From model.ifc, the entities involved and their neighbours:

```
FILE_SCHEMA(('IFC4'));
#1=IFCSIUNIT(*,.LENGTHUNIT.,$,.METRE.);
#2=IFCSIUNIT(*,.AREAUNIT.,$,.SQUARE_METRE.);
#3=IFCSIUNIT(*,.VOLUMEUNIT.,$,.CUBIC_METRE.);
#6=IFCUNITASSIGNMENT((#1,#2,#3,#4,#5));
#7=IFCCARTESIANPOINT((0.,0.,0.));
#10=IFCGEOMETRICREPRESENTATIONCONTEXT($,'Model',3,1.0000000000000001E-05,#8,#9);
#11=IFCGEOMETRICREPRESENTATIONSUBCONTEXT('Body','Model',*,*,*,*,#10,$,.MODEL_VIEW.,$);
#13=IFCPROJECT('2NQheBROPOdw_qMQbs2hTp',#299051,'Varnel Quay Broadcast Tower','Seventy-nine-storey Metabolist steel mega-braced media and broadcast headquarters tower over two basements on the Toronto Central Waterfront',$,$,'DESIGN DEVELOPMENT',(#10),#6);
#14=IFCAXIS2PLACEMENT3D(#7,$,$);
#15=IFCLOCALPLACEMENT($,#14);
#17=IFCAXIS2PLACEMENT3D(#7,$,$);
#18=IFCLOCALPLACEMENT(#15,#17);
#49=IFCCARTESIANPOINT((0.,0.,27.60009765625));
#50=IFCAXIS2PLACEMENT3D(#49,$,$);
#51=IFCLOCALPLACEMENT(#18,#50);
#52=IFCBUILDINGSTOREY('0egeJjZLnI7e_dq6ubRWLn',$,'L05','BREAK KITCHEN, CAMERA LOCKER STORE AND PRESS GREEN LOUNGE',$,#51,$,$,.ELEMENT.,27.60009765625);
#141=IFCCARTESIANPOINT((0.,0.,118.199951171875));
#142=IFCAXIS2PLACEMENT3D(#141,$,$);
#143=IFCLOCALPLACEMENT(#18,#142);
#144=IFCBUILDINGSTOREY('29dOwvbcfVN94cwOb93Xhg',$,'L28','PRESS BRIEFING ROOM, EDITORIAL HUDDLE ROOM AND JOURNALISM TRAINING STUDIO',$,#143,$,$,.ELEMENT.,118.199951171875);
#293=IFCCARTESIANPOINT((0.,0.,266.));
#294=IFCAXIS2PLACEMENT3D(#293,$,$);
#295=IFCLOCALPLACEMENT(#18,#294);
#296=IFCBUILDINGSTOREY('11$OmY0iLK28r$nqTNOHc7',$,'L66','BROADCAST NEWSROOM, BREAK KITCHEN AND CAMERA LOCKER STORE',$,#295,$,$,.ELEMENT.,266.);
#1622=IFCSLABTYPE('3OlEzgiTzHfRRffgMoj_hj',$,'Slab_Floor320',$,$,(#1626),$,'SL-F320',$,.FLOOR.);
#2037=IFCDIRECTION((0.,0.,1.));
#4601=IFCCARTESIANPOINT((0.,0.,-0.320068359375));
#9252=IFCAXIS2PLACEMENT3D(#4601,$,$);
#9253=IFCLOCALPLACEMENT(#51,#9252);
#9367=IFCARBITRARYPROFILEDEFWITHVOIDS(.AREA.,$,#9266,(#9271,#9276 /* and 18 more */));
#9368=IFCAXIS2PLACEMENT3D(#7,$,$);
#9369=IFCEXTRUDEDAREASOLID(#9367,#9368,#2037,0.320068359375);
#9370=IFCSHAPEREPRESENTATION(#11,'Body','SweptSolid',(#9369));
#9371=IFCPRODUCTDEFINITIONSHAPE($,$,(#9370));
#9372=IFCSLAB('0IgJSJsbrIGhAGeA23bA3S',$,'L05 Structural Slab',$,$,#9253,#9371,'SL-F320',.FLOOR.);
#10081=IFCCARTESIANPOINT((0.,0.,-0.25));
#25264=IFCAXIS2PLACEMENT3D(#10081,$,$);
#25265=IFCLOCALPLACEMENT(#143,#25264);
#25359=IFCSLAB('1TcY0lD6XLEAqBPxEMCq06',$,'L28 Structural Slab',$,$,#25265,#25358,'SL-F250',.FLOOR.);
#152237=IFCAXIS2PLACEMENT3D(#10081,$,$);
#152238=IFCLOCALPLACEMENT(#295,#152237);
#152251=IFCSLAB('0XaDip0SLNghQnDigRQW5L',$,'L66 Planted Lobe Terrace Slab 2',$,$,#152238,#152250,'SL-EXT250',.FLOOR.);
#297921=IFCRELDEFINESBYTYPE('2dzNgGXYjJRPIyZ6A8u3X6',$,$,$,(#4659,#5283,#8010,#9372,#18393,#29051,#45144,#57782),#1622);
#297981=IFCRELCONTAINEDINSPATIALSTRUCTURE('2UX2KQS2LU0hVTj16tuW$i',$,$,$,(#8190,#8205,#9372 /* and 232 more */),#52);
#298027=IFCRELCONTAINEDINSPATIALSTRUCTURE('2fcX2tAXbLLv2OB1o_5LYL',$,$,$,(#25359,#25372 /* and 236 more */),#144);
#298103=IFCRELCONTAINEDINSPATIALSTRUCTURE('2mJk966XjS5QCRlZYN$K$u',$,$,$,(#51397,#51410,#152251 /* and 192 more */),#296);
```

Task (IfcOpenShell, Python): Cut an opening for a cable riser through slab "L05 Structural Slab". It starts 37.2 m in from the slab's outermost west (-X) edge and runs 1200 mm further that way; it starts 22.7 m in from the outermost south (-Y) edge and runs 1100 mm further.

```python
import numpy as np
import ifcopenshell
import ifcopenshell.api.feature
import ifcopenshell.api.geometry
import ifcopenshell.api.root
import ifcopenshell.geom
import ifcopenshell.util.placement
import ifcopenshell.util.representation
import ifcopenshell.util.shape
import ifcopenshell.util.unit

model = ifcopenshell.open("model.ifc")
unit_scale = ifcopenshell.util.unit.calculate_unit_scale(model)
settings = ifcopenshell.geom.settings()


def volume(element):
    """Net volume in cubic metres, openings subtracted."""
    shape = ifcopenshell.geom.create_shape(settings, element)
    return ifcopenshell.util.shape.get_volume(shape.geometry)


slab = model.by_guid("0IgJSJsbrIGhAGeA23bA3S")
before = volume(slab)

# Extent in the slab's own axes, in metres. The edges named are its -X and -Y sides.
slab_shape = ifcopenshell.geom.create_shape(settings, slab)
vertices = ifcopenshell.util.shape.get_vertices(slab_shape.geometry)
x_min, y_min, bottom = vertices.min(axis=0)
top = vertices[:, 2].max()

opening = ifcopenshell.api.root.create_entity(model, ifc_class="IfcOpeningElement", name="Cable riser opening", predefined_type="OPENING")
context = ifcopenshell.util.representation.get_context(model, "Model", "Body", "MODEL_VIEW")
width, depth = 1.2, 1.1
outline = [(0.0, 0.0), (width, 0.0), (width, depth), (0.0, depth), (0.0, 0.0)]
# Overshoot both faces by 50 mm so the cut is clean.
shape = ifcopenshell.api.geometry.add_slab_representation(
    model, context=context, depth=top - bottom + 0.1, polyline=outline
)
ifcopenshell.api.geometry.assign_representation(model, product=opening, representation=shape)

matrix = ifcopenshell.util.placement.get_local_placement(slab.ObjectPlacement)
matrix[:, 3] = matrix @ np.append(np.array([x_min + 37.2, y_min + 22.7, bottom - 0.05]) / unit_scale, 1.0)
ifcopenshell.api.geometry.edit_object_placement(model, product=opening, matrix=matrix, is_si=False)
ifcopenshell.api.feature.add_feature(model, feature=opening, element=slab)

after = volume(slab)

print(f"slab volume {before:.3f} -> {after:.3f} m3")

model.write("model-out.ifc")
```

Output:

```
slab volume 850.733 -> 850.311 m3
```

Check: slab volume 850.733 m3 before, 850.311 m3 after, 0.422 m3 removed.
